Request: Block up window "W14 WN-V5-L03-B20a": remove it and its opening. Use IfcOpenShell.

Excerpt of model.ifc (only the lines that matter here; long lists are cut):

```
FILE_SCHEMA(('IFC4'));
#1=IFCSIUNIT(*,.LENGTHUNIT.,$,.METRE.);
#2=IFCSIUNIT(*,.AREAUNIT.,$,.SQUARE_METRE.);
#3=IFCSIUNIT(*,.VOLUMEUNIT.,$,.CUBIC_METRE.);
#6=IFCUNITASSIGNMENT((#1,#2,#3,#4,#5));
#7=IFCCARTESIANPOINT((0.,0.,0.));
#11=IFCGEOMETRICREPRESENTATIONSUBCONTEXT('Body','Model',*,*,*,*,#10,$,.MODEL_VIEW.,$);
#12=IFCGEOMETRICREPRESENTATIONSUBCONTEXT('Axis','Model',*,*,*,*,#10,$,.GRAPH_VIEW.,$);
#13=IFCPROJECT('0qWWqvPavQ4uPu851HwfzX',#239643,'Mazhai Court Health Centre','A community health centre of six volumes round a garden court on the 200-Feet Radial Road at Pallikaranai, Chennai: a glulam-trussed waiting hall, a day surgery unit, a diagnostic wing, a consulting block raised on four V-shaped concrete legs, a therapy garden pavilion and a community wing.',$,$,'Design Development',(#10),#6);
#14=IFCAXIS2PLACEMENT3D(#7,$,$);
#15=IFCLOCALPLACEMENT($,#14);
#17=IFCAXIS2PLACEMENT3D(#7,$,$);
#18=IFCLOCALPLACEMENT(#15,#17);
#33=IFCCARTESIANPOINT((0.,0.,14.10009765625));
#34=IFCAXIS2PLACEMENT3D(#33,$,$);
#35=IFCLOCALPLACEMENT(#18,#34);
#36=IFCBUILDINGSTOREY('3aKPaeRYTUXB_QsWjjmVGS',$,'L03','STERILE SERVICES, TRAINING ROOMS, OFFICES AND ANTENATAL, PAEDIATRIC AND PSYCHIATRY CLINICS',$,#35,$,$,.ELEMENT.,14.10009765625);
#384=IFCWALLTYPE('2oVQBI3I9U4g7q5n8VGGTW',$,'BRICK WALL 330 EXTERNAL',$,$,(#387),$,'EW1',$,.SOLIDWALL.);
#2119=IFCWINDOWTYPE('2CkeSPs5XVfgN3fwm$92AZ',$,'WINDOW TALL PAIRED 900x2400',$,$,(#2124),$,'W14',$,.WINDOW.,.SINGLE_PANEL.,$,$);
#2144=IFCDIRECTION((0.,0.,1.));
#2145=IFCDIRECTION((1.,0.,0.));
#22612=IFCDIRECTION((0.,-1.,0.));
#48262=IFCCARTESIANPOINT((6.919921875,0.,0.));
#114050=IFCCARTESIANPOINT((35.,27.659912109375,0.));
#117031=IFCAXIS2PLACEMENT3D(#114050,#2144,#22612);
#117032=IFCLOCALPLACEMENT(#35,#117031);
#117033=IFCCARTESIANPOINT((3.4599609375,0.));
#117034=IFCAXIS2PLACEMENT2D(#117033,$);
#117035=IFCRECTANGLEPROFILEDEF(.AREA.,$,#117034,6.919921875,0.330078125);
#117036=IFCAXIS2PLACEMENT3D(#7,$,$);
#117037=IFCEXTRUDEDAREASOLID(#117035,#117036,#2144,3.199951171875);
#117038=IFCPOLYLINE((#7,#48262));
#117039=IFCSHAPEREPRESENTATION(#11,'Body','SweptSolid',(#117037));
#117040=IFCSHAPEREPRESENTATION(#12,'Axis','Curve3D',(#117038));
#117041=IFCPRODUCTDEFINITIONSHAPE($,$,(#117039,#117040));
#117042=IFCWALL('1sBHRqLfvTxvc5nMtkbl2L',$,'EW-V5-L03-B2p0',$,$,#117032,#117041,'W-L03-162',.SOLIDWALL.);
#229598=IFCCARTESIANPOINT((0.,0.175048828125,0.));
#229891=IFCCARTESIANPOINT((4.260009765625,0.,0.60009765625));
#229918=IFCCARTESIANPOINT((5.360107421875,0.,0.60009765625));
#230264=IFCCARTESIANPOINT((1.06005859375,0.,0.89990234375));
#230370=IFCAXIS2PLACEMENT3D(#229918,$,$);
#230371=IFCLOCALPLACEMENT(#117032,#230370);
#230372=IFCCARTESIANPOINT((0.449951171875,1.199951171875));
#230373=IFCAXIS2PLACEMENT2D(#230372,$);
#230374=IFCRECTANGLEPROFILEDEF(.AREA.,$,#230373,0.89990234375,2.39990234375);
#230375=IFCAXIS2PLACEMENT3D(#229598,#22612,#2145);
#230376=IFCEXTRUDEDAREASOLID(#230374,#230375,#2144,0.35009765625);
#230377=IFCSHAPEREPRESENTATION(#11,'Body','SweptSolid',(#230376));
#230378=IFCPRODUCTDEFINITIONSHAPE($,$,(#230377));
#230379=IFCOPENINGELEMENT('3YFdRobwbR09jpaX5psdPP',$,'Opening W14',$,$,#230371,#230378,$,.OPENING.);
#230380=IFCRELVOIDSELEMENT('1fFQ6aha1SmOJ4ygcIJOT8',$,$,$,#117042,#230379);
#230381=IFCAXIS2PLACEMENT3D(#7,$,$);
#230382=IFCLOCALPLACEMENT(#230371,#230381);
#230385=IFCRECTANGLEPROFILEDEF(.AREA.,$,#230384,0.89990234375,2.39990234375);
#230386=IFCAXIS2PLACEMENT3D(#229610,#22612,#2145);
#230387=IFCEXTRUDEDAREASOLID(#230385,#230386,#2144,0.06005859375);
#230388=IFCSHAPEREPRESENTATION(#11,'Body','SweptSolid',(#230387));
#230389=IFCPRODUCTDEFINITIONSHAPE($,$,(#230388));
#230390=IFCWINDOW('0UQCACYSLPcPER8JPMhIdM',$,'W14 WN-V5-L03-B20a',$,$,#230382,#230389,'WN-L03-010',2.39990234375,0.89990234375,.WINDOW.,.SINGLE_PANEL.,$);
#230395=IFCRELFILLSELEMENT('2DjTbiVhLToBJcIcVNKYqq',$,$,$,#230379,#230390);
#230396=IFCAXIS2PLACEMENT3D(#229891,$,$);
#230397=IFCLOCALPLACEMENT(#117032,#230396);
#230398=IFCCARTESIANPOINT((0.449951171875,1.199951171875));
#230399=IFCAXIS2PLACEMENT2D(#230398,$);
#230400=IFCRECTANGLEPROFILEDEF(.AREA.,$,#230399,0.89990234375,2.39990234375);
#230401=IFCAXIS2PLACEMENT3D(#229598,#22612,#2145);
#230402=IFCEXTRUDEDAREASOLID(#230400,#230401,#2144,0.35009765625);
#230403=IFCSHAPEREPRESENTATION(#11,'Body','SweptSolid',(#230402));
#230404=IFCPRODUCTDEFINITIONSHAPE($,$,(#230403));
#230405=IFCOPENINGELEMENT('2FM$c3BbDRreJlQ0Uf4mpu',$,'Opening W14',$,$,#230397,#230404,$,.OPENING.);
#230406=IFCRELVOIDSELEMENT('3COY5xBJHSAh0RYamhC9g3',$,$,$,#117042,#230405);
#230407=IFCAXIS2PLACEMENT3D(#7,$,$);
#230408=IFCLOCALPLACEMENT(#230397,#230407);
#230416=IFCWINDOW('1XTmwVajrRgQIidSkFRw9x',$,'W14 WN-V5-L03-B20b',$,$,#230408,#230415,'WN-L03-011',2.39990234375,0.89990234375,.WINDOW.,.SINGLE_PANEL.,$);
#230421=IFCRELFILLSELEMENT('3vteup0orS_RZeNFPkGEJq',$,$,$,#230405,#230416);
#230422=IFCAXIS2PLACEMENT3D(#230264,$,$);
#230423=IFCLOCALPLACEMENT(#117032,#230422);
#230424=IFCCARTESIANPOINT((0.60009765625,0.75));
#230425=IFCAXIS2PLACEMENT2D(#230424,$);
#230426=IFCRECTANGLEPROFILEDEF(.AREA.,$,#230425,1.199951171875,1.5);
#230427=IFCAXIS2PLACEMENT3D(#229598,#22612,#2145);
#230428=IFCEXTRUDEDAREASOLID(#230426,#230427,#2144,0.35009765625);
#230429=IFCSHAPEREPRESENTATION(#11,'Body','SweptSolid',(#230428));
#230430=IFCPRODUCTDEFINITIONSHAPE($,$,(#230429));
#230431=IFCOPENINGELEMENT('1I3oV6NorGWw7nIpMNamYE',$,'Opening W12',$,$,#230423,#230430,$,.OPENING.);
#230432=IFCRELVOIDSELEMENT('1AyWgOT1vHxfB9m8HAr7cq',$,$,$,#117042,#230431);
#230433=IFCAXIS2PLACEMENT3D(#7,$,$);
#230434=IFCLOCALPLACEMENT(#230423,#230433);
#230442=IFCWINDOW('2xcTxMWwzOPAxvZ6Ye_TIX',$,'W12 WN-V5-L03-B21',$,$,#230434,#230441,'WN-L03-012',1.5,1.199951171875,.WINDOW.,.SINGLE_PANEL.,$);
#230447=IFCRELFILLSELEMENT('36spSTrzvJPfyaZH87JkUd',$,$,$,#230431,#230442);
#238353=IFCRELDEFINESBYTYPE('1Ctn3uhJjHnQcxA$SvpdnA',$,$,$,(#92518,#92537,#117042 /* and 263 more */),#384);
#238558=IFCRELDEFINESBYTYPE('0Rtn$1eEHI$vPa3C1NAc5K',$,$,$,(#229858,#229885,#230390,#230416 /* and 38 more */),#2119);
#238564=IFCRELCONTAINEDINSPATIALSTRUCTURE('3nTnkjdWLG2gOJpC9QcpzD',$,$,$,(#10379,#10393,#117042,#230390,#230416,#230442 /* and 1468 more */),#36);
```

```python
import ifcopenshell
import ifcopenshell.api.feature
import ifcopenshell.api.root
import ifcopenshell.geom
import ifcopenshell.util.shape

model = ifcopenshell.open("model.ifc")
settings = ifcopenshell.geom.settings()


def volume(element):
    """Net volume in cubic metres, openings subtracted."""
    shape = ifcopenshell.geom.create_shape(settings, element)
    return ifcopenshell.util.shape.get_volume(shape.geometry)


window = model.by_guid("0UQCACYSLPcPER8JPMhIdM")
opening = window.FillsVoids[0].RelatingOpeningElement
wall = opening.VoidsElements[0].RelatingBuildingElement
before = volume(wall)

ifcopenshell.api.root.remove_product(model, product=window)
ifcopenshell.api.feature.remove_feature(model, feature=opening)

after = volume(wall)

print(f"wall volume {before:.3f} -> {after:.3f} m3")

model.write("model_rev.ifc")
```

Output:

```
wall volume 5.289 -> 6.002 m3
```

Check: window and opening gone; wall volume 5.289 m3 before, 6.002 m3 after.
